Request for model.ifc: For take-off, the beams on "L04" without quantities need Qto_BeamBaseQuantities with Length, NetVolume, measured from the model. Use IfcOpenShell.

First a look at what the model holds.

```python
import ifcopenshell
import ifcopenshell.util.element
import ifcopenshell.util.unit

model = ifcopenshell.open("model.ifc")
print(model.schema)
for unit_type in ("LENGTHUNIT", "AREAUNIT", "VOLUMEUNIT"):
    print(unit_type, ifcopenshell.util.unit.calculate_unit_scale(model, unit_type))
storey = next(s for s in model.by_type("IfcBuildingStorey") if s.Name == "L04")
beams = [e for e in ifcopenshell.util.element.get_decomposition(storey) if e.is_a("IfcBeam")]
for e in sorted(beams, key=lambda e: e.id()):
    print(e.id(), e.is_a(), e.Name, list(ifcopenshell.util.element.get_psets(e, qtos_only=True)), sep=" | ")
```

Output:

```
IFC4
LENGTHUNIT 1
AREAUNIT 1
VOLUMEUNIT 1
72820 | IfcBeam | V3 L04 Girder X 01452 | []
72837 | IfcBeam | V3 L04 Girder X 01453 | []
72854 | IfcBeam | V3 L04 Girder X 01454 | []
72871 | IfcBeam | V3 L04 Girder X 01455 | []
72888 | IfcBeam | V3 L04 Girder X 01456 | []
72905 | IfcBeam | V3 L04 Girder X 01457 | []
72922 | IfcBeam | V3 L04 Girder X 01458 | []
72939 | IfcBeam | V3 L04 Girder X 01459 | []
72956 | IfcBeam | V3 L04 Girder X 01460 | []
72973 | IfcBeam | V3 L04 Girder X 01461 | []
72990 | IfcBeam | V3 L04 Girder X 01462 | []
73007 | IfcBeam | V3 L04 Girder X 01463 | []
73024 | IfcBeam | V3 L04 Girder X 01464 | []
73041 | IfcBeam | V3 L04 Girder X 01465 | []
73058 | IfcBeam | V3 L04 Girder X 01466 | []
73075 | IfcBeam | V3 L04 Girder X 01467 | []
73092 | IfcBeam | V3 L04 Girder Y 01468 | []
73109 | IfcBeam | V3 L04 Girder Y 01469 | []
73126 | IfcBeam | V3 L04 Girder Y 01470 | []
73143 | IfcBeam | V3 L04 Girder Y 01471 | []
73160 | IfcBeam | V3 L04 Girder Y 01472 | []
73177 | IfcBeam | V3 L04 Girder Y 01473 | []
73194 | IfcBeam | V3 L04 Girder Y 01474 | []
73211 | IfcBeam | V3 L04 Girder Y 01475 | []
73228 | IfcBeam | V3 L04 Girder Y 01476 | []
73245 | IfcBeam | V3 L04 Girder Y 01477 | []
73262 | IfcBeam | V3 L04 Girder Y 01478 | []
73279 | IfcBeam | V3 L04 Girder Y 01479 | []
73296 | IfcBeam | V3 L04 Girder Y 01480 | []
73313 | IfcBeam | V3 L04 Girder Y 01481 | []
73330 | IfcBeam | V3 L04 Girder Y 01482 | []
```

```python
import ifcopenshell
import ifcopenshell.api.pset
import ifcopenshell.geom
import ifcopenshell.util.element
import ifcopenshell.util.shape
import ifcopenshell.util.unit

model = ifcopenshell.open("model.ifc")
unit_scale = ifcopenshell.util.unit.calculate_unit_scale(model)
volume_scale = ifcopenshell.util.unit.calculate_unit_scale(model, "VOLUMEUNIT")
settings = ifcopenshell.geom.settings()

storey = next(s for s in model.by_type("IfcBuildingStorey") if s.Name == "L04")
beams = [e for e in ifcopenshell.util.element.get_decomposition(storey) if e.is_a("IfcBeam")]

for e in sorted(beams, key=lambda e: e.id()):
    if ifcopenshell.util.element.get_psets(e, qtos_only=True, should_inherit=False):
        continue
    # Geometry comes back in metres, in the element's own axes.
    shape = ifcopenshell.geom.create_shape(settings, e)
    values = {
        "Length": ifcopenshell.util.shape.get_max_xyz(shape.geometry) / unit_scale,
        "NetVolume": ifcopenshell.util.shape.get_volume(shape.geometry) / volume_scale,
    }
    qto = ifcopenshell.api.pset.add_qto(model, product=e, name="Qto_BeamBaseQuantities")
    ifcopenshell.api.pset.edit_qto(model, qto=qto, properties=values)
    print(e.id(), {k: round(v, 3) for k, v in values.items()})

model.write("model_updated.ifc")
```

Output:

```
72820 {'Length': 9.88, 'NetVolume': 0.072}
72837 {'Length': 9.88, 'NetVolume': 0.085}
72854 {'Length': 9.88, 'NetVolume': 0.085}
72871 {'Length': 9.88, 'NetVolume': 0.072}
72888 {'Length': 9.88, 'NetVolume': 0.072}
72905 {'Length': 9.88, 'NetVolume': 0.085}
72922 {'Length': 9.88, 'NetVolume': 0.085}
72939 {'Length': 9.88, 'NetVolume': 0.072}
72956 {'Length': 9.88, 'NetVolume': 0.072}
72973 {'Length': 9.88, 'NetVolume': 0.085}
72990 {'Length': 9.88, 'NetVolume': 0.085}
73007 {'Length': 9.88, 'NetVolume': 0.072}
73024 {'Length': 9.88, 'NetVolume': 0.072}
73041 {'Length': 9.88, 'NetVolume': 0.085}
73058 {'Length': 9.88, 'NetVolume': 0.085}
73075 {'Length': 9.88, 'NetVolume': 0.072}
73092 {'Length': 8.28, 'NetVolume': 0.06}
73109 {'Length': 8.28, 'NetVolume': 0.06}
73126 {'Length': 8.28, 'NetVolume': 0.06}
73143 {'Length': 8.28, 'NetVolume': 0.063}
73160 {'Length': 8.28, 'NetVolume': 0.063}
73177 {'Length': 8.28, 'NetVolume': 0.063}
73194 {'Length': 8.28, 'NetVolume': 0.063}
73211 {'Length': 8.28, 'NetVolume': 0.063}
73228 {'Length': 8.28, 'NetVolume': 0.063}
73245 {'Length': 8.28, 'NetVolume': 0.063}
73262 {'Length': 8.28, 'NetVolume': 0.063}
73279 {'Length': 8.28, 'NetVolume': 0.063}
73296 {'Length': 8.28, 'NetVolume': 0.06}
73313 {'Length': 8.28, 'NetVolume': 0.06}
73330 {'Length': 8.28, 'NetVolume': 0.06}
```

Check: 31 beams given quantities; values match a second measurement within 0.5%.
